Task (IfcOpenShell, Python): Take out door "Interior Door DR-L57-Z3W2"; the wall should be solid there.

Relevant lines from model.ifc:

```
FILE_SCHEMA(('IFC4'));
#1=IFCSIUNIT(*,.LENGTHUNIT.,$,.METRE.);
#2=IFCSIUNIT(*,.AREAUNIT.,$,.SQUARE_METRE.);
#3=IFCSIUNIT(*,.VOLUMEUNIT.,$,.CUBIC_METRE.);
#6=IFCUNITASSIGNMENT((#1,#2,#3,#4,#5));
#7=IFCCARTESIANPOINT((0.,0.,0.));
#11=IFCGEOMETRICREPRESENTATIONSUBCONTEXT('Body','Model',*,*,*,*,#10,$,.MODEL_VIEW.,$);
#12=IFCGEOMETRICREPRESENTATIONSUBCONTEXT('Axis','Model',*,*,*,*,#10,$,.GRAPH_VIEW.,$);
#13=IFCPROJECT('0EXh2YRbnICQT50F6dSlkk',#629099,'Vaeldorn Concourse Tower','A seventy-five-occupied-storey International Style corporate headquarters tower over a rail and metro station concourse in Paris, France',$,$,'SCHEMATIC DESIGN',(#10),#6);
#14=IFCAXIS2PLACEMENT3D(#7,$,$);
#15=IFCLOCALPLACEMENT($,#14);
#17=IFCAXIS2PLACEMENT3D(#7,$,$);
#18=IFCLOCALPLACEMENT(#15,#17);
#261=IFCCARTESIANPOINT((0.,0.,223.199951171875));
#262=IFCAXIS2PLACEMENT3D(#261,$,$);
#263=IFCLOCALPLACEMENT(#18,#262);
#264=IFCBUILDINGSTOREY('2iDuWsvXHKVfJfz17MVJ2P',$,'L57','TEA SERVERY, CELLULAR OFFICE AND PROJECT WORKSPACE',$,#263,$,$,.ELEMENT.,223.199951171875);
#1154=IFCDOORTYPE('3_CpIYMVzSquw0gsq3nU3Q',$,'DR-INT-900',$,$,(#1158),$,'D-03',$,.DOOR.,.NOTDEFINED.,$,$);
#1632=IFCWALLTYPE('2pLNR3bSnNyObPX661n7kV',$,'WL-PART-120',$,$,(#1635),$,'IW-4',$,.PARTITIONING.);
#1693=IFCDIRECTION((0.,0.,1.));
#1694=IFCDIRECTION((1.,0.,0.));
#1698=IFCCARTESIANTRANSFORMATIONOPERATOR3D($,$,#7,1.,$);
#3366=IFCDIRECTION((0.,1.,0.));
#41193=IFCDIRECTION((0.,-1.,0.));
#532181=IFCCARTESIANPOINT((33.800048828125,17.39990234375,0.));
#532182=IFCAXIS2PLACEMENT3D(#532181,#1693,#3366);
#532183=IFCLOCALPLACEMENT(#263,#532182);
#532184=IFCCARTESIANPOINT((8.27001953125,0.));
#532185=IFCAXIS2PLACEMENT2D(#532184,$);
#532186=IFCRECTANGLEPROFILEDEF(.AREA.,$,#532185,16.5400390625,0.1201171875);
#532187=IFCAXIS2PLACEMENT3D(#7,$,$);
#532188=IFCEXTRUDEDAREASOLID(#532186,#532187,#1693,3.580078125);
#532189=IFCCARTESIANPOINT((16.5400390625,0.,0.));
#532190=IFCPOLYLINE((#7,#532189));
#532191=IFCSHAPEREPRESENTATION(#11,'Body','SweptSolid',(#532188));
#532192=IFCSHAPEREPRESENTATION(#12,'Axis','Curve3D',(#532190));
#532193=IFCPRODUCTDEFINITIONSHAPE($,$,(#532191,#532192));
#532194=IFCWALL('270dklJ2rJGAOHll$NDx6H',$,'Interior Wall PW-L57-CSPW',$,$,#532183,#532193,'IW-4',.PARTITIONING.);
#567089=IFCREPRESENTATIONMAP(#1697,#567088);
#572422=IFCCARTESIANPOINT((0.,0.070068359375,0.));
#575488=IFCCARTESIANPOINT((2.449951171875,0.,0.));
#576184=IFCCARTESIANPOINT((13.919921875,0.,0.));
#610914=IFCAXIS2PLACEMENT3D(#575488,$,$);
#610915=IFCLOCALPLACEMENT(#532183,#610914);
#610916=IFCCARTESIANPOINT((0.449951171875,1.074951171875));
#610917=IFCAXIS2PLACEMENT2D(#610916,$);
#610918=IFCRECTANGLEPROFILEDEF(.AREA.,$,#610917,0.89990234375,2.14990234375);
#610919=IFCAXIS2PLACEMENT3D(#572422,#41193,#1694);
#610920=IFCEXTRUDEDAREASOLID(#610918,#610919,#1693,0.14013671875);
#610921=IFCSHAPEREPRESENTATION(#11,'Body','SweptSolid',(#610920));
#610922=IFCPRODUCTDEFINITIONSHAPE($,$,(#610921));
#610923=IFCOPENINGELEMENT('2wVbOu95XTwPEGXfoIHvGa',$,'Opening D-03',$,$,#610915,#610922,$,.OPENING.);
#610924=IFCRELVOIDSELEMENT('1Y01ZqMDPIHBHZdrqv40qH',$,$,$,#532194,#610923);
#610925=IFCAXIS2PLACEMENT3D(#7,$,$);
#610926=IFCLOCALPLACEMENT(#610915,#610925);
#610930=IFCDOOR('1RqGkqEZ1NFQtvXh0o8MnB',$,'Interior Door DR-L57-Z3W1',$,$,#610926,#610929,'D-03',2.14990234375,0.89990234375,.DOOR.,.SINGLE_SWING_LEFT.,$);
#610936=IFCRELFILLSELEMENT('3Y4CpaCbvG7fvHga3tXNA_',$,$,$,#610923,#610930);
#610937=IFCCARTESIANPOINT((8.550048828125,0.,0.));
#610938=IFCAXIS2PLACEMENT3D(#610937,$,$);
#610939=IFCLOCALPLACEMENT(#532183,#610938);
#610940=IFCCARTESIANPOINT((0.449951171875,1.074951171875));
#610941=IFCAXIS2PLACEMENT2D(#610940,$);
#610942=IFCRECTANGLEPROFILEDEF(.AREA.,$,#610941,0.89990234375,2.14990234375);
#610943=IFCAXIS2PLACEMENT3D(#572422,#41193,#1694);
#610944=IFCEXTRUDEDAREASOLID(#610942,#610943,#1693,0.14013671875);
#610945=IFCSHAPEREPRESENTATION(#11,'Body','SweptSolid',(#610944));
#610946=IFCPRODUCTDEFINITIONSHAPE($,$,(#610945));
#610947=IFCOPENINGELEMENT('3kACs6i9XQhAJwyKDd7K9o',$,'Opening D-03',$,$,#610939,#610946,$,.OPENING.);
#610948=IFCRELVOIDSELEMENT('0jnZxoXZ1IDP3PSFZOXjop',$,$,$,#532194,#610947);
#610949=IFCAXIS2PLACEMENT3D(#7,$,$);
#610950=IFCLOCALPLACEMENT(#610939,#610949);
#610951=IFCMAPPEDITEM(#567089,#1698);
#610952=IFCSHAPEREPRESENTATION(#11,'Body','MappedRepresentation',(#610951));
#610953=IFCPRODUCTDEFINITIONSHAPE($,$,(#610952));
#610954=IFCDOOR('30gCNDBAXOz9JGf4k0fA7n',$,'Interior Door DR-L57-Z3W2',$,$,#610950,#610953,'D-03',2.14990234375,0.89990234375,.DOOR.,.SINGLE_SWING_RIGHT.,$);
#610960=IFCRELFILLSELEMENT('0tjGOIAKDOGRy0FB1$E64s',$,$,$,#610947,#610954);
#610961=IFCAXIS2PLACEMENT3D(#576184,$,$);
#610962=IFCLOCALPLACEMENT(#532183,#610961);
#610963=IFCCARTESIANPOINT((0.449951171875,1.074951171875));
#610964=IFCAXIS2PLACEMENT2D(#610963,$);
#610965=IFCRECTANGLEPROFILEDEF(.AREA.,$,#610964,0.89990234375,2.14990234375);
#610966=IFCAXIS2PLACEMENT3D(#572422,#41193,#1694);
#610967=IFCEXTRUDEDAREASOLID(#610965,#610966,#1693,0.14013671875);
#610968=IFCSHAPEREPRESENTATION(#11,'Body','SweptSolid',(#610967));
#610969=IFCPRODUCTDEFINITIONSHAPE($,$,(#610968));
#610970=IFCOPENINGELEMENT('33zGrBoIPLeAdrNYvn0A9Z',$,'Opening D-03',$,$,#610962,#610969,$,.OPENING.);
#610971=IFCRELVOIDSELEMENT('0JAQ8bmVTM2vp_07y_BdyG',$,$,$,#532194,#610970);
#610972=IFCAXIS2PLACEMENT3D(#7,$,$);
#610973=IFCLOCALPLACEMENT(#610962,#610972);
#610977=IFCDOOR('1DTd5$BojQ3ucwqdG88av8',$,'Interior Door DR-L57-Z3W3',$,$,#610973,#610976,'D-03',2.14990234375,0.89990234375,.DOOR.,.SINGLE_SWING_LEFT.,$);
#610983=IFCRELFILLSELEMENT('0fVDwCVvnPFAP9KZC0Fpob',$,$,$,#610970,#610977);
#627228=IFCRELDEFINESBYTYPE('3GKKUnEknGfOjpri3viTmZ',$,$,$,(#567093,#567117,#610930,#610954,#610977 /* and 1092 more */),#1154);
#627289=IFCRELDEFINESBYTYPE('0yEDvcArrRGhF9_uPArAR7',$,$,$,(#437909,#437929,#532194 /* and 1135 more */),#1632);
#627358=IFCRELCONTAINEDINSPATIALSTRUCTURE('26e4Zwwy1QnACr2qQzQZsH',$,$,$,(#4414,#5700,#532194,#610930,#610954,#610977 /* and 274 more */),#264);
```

```python
import ifcopenshell
import ifcopenshell.api.feature
import ifcopenshell.api.root
import ifcopenshell.geom
import ifcopenshell.util.shape

model = ifcopenshell.open("model.ifc")
settings = ifcopenshell.geom.settings()


def volume(element):
    """Net volume in cubic metres, openings subtracted."""
    shape = ifcopenshell.geom.create_shape(settings, element)
    return ifcopenshell.util.shape.get_volume(shape.geometry)


door = model.by_guid("30gCNDBAXOz9JGf4k0fA7n")
opening = door.FillsVoids[0].RelatingOpeningElement
wall = opening.VoidsElements[0].RelatingBuildingElement
before = volume(wall)

ifcopenshell.api.root.remove_product(model, product=door)
ifcopenshell.api.feature.remove_feature(model, feature=opening)

after = volume(wall)

print(f"wall volume {before:.3f} -> {after:.3f} m3")

model.write("model-out.ifc")
```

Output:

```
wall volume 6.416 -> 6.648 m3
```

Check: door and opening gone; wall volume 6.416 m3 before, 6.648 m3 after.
